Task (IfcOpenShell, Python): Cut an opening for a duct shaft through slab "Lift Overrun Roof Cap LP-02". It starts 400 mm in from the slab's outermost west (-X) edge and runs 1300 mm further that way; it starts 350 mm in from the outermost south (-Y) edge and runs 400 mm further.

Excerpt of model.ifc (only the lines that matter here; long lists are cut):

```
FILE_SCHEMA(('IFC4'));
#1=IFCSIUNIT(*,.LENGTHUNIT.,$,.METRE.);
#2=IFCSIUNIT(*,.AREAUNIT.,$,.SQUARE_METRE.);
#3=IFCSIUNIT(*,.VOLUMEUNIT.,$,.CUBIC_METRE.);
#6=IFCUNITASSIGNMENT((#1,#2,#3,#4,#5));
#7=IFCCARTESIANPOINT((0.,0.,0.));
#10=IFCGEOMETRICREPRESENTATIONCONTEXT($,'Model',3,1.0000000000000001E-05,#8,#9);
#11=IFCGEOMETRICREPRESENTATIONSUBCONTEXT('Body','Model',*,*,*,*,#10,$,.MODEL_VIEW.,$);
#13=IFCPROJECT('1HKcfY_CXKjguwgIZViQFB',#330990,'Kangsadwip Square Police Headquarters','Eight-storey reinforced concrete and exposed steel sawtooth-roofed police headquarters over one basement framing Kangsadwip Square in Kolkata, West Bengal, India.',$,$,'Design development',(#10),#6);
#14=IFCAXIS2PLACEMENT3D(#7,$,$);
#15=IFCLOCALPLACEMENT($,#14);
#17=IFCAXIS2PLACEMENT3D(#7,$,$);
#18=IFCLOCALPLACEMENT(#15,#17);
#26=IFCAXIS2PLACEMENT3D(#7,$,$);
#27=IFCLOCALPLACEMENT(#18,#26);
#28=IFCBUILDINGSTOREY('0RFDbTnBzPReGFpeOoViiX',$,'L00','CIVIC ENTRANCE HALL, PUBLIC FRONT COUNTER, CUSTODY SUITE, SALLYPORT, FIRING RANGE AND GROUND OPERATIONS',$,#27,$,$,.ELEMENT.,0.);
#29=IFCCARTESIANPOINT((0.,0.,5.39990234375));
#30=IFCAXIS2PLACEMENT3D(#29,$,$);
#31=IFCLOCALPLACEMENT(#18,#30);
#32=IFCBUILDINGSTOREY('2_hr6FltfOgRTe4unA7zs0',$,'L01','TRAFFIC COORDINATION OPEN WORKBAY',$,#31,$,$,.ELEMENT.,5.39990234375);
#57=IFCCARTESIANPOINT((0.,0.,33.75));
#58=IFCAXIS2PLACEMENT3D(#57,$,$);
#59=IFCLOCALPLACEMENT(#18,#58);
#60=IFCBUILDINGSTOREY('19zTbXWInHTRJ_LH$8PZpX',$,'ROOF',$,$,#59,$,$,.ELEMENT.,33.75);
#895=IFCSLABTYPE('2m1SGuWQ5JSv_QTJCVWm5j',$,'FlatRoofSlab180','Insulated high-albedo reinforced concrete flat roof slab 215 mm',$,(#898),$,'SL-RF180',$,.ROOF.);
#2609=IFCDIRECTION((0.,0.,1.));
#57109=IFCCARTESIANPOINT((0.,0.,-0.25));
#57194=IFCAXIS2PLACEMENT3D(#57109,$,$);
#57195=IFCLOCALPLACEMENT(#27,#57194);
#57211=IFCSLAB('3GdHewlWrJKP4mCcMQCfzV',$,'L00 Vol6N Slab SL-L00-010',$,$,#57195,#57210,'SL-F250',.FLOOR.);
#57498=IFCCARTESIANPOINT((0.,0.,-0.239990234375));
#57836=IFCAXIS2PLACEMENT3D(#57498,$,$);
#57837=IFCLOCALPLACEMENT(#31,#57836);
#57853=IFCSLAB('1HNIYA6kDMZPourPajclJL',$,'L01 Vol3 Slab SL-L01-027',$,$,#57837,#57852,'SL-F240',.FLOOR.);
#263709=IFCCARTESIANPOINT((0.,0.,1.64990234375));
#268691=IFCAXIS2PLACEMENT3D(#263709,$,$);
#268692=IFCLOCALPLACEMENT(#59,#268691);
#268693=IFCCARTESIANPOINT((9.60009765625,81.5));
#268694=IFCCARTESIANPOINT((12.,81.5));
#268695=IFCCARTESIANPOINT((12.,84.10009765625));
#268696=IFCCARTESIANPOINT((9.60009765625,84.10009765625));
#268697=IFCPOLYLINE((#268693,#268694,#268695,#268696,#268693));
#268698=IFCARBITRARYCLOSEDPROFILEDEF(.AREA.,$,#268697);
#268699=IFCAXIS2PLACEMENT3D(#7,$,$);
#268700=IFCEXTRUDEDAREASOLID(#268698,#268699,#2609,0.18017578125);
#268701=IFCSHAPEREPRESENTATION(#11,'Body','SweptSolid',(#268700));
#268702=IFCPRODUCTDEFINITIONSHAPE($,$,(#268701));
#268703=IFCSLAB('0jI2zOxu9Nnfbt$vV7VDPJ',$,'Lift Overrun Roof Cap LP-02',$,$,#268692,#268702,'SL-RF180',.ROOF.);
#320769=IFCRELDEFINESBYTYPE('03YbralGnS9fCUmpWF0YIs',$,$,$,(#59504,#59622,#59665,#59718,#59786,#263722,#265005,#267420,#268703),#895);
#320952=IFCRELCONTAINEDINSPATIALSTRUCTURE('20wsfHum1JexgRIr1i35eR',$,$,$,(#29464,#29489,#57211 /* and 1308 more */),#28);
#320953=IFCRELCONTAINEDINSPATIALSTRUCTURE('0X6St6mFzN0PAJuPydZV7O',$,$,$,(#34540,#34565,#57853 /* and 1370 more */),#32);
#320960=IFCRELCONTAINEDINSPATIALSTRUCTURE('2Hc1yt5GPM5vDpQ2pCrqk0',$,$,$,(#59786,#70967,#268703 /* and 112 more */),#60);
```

```python
import numpy as np
import ifcopenshell
import ifcopenshell.api.feature
import ifcopenshell.api.geometry
import ifcopenshell.api.root
import ifcopenshell.geom
import ifcopenshell.util.placement
import ifcopenshell.util.representation
import ifcopenshell.util.shape
import ifcopenshell.util.unit

model = ifcopenshell.open("model.ifc")
unit_scale = ifcopenshell.util.unit.calculate_unit_scale(model)
settings = ifcopenshell.geom.settings()


def volume(element):
    """Net volume in cubic metres, openings subtracted."""
    shape = ifcopenshell.geom.create_shape(settings, element)
    return ifcopenshell.util.shape.get_volume(shape.geometry)


slab = model.by_id(268703)
before = volume(slab)

# Extent in the slab's own axes, in metres. The edges named are its -X and -Y sides.
slab_shape = ifcopenshell.geom.create_shape(settings, slab)
vertices = ifcopenshell.util.shape.get_vertices(slab_shape.geometry)
x_min, y_min, bottom = vertices.min(axis=0)
top = vertices[:, 2].max()

opening = ifcopenshell.api.root.create_entity(model, ifc_class="IfcOpeningElement", name="Duct shaft opening", predefined_type="OPENING")
context = ifcopenshell.util.representation.get_context(model, "Model", "Body", "MODEL_VIEW")
width, depth = 1.3, 0.4
outline = [(0.0, 0.0), (width, 0.0), (width, depth), (0.0, depth), (0.0, 0.0)]
# Overshoot both faces by 50 mm so the cut is clean.
shape = ifcopenshell.api.geometry.add_slab_representation(
    model, context=context, depth=top - bottom + 0.1, polyline=outline
)
ifcopenshell.api.geometry.assign_representation(model, product=opening, representation=shape)

matrix = ifcopenshell.util.placement.get_local_placement(slab.ObjectPlacement)
matrix[:, 3] = matrix @ np.append(np.array([x_min + 0.4, y_min + 0.35, bottom - 0.05]) / unit_scale, 1.0)
ifcopenshell.api.geometry.edit_object_placement(model, product=opening, matrix=matrix, is_si=False)
ifcopenshell.api.feature.add_feature(model, feature=opening, element=slab)

after = volume(slab)

print(f"slab volume {before:.3f} -> {after:.3f} m3")

model.write("model-out.ifc")
```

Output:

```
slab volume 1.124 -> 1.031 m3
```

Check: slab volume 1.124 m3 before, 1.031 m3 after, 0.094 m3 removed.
